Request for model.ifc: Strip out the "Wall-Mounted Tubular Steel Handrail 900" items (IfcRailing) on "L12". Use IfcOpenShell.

First a look at what the model holds.

```python
import ifcopenshell
import ifcopenshell.util.element

model = ifcopenshell.open("model.ifc")
print(model.schema)
storey = next(s for s in model.by_type("IfcBuildingStorey") if s.Name == "L12")
railings = [e for e in ifcopenshell.util.element.get_decomposition(storey) if e.is_a("IfcRailing")]
seen = {}
for e in railings:
    element_type = ifcopenshell.util.element.get_type(e)
    name = element_type.Name if element_type not in (None, e) else None
    seen[name] = seen.get(name, 0) + 1
for name, count in sorted(seen.items(), key=str):
    print(count, "x", name)
```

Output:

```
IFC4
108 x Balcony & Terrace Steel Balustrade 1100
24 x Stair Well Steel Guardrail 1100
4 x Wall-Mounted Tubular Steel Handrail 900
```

```python
import ifcopenshell
import ifcopenshell.api.root
import ifcopenshell.util.element

model = ifcopenshell.open("model.ifc")

storey = next(s for s in model.by_type("IfcBuildingStorey") if s.Name == "L12")
railings = [e for e in ifcopenshell.util.element.get_decomposition(storey) if e.is_a("IfcRailing")]
targets = [e for e in railings if (t := ifcopenshell.util.element.get_type(e)) not in (None, e) and t.Name == "Wall-Mounted Tubular Steel Handrail 900"]

for e in targets:
    ifcopenshell.api.root.remove_product(model, product=e)
print(len(targets), "removed")

model.write("model_updated.ifc")
```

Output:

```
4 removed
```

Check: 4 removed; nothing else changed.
